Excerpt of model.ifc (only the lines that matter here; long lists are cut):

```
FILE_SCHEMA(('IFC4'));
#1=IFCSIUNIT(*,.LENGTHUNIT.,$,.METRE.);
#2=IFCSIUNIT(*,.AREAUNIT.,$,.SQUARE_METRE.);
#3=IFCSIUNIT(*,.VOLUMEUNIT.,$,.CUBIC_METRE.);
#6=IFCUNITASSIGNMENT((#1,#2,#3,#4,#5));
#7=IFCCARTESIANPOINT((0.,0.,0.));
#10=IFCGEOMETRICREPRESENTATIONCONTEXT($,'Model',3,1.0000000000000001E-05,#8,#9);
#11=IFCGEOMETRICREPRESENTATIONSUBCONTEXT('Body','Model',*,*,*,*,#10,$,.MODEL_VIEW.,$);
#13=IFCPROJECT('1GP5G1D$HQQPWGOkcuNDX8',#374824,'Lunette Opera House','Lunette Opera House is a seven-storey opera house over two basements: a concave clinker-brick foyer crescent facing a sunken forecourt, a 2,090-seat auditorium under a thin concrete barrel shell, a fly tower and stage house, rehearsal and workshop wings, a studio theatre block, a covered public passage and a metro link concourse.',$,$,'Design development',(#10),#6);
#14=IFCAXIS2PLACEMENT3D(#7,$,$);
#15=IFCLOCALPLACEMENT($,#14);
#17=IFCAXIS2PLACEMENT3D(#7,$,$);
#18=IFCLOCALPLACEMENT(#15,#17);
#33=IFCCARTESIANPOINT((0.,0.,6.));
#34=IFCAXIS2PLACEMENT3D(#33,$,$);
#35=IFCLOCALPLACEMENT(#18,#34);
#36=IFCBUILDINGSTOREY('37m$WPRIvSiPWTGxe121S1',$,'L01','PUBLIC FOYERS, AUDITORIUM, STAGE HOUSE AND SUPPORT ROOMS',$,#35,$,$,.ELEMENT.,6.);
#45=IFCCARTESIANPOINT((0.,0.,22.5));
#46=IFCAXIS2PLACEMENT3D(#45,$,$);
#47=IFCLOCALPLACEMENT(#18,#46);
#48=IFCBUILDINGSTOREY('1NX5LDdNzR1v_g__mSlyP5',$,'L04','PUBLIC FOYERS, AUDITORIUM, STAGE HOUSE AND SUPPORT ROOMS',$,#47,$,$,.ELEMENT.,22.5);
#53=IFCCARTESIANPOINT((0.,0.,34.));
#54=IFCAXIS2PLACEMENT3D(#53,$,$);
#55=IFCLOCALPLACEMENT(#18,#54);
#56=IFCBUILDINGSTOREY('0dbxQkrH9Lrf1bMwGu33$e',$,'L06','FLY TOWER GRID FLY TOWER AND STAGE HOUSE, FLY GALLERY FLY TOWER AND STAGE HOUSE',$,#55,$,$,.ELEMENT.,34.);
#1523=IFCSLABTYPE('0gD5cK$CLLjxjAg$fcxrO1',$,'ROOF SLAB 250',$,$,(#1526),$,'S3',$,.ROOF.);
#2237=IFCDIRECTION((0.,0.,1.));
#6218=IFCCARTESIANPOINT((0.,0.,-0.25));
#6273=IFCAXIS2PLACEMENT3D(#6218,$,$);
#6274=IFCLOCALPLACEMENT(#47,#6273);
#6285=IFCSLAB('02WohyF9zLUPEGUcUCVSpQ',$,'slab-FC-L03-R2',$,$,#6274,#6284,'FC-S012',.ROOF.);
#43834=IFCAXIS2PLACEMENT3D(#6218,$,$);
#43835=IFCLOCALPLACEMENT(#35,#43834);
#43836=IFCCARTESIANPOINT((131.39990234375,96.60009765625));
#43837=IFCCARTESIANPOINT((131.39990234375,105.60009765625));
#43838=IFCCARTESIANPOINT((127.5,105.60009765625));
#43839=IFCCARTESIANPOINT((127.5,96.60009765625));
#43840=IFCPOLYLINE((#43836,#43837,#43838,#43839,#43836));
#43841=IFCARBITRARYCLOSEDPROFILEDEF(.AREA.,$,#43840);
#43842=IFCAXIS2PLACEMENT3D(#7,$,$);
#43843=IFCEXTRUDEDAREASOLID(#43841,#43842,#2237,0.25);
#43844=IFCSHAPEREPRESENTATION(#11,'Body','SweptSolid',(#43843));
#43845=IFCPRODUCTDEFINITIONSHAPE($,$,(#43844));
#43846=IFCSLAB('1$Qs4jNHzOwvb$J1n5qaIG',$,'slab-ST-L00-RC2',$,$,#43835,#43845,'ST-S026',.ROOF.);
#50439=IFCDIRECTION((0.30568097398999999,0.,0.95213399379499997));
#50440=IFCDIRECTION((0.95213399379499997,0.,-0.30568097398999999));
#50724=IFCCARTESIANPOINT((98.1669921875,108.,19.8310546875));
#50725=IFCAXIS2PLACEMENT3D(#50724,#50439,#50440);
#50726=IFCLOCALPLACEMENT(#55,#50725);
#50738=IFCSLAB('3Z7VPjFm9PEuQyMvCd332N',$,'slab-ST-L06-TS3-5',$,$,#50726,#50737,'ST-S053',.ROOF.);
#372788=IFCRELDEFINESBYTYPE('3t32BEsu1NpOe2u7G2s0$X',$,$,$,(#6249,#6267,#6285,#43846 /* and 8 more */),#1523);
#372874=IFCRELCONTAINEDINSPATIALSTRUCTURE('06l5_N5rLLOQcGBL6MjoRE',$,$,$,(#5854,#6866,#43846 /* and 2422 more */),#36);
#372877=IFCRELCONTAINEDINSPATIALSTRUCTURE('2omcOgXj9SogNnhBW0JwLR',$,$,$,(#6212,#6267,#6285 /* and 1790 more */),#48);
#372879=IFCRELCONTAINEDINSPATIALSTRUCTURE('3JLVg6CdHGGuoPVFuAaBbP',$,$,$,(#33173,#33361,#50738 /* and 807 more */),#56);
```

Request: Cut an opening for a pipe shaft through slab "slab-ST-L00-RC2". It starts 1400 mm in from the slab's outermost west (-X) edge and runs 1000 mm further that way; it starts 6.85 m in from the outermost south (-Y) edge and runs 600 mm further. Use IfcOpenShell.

```python
import numpy as np
import ifcopenshell
import ifcopenshell.api.feature
import ifcopenshell.api.geometry
import ifcopenshell.api.root
import ifcopenshell.geom
import ifcopenshell.util.placement
import ifcopenshell.util.representation
import ifcopenshell.util.shape
import ifcopenshell.util.unit

model = ifcopenshell.open("model.ifc")
unit_scale = ifcopenshell.util.unit.calculate_unit_scale(model)
settings = ifcopenshell.geom.settings()


def volume(element):
    """Net volume in cubic metres, openings subtracted."""
    shape = ifcopenshell.geom.create_shape(settings, element)
    return ifcopenshell.util.shape.get_volume(shape.geometry)


slab = model.by_guid("1$Qs4jNHzOwvb$J1n5qaIG")
before = volume(slab)

# Extent in the slab's own axes, in metres. The edges named are its -X and -Y sides.
slab_shape = ifcopenshell.geom.create_shape(settings, slab)
vertices = ifcopenshell.util.shape.get_vertices(slab_shape.geometry)
x_min, y_min, bottom = vertices.min(axis=0)
top = vertices[:, 2].max()

opening = ifcopenshell.api.root.create_entity(model, ifc_class="IfcOpeningElement", name="Pipe shaft opening", predefined_type="OPENING")
context = ifcopenshell.util.representation.get_context(model, "Model", "Body", "MODEL_VIEW")
width, depth = 1, 0.6
outline = [(0.0, 0.0), (width, 0.0), (width, depth), (0.0, depth), (0.0, 0.0)]
# Overshoot both faces by 50 mm so the cut is clean.
shape = ifcopenshell.api.geometry.add_slab_representation(
    model, context=context, depth=top - bottom + 0.1, polyline=outline
)
ifcopenshell.api.geometry.assign_representation(model, product=opening, representation=shape)

matrix = ifcopenshell.util.placement.get_local_placement(slab.ObjectPlacement)
matrix[:, 3] = matrix @ np.append(np.array([x_min + 1.4, y_min + 6.85, bottom - 0.05]) / unit_scale, 1.0)
ifcopenshell.api.geometry.edit_object_placement(model, product=opening, matrix=matrix, is_si=False)
ifcopenshell.api.feature.add_feature(model, feature=opening, element=slab)

after = volume(slab)

print(f"slab volume {before:.3f} -> {after:.3f} m3")

model.write("model_edited.ifc")
```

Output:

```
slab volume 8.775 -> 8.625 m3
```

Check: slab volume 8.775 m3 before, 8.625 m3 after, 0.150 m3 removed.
